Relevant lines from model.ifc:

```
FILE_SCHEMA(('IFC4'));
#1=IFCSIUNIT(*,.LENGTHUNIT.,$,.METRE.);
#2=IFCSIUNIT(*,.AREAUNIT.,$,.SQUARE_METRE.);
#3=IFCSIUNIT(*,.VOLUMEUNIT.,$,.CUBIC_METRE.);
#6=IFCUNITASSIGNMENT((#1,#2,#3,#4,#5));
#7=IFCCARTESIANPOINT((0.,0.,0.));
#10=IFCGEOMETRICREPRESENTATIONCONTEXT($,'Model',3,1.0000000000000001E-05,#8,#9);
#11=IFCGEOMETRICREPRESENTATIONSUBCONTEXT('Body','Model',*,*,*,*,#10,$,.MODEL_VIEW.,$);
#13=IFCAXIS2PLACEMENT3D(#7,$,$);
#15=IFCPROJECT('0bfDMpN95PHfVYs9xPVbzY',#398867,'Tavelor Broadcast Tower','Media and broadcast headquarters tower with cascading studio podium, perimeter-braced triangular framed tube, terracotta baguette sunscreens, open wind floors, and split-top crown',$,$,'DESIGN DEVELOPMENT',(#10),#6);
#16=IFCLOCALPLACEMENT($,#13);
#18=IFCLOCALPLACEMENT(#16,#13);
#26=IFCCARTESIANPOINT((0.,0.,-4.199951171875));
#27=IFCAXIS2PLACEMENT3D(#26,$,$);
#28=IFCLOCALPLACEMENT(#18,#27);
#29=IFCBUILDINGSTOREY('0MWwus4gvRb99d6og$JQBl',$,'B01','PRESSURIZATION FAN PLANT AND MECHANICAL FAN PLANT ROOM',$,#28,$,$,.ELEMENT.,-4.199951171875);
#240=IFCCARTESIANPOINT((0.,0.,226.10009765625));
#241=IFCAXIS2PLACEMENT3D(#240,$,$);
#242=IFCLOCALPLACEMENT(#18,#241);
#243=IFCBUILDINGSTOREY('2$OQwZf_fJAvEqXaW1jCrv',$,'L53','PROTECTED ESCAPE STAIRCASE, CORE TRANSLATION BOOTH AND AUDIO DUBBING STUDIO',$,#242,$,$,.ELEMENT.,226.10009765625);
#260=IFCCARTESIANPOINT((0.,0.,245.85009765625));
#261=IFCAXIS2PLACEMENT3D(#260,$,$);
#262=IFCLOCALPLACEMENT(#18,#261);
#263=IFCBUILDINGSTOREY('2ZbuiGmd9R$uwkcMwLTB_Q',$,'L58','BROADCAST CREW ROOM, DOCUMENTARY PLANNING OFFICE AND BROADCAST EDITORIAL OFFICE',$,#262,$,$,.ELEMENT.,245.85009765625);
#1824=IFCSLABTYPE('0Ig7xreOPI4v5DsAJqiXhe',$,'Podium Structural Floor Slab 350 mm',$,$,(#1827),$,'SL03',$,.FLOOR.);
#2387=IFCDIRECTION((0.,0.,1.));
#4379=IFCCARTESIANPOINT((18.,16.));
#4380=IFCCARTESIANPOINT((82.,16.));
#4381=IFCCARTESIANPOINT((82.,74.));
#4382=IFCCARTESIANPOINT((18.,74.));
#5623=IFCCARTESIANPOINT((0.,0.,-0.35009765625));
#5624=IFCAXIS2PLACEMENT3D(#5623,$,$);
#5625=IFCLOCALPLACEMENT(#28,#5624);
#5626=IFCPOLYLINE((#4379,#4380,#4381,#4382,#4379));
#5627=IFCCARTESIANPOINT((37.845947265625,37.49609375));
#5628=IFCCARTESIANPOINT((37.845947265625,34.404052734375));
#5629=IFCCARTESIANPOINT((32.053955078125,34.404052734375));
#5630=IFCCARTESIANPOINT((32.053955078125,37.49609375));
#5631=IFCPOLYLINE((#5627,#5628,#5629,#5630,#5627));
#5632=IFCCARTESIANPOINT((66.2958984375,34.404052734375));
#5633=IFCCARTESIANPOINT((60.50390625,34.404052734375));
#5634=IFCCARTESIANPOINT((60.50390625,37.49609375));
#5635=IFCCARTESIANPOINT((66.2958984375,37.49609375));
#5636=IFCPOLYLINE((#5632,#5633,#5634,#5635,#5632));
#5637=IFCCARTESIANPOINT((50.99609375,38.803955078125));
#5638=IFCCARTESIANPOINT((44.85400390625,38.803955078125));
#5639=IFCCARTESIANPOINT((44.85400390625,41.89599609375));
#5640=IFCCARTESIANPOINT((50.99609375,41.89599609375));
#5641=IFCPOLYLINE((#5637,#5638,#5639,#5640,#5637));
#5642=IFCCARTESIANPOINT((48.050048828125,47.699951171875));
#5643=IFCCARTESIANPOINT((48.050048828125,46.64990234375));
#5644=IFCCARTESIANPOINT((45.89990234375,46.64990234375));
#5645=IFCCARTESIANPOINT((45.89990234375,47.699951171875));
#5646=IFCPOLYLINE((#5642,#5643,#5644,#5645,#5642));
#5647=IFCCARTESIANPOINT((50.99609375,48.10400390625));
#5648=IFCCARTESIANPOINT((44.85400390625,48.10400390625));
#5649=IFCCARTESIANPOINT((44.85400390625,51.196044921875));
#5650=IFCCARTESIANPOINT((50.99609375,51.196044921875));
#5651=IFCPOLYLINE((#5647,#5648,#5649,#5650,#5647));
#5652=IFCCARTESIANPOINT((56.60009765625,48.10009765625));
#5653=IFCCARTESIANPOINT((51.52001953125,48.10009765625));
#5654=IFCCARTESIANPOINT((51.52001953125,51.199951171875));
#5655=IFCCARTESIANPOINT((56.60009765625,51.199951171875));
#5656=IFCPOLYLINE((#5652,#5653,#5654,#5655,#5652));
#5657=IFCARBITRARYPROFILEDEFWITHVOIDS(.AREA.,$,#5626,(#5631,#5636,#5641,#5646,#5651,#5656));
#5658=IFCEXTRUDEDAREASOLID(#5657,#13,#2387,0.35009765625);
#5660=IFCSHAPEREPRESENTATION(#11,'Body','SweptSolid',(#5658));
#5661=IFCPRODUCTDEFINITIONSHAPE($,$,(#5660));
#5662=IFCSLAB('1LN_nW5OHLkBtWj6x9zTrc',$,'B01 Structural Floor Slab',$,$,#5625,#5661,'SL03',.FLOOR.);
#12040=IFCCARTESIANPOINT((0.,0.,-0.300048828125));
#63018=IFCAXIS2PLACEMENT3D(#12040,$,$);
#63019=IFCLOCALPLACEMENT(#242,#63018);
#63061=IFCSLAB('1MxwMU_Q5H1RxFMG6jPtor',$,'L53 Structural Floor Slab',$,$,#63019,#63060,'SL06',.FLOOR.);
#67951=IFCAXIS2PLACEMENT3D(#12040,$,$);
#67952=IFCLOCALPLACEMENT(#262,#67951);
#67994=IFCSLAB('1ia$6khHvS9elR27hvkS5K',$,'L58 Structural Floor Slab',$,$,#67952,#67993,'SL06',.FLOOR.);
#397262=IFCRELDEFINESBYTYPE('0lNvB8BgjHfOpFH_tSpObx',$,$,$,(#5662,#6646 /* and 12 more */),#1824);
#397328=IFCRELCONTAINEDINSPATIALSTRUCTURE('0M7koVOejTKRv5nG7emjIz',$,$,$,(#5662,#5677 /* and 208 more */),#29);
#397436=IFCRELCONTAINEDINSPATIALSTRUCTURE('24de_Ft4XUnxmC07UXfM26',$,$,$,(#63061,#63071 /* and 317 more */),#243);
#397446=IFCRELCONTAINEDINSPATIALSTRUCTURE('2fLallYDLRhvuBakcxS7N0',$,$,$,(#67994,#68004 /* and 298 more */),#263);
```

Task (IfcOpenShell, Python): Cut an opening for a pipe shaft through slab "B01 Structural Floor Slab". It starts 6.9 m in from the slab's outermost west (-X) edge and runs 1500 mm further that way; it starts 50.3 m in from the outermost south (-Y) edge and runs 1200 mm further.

```python
import numpy as np
import ifcopenshell
import ifcopenshell.api.feature
import ifcopenshell.api.geometry
import ifcopenshell.api.root
import ifcopenshell.geom
import ifcopenshell.util.placement
import ifcopenshell.util.representation
import ifcopenshell.util.shape
import ifcopenshell.util.unit

model = ifcopenshell.open("model.ifc")
unit_scale = ifcopenshell.util.unit.calculate_unit_scale(model)
settings = ifcopenshell.geom.settings()


def volume(element):
    """Net volume in cubic metres, openings subtracted."""
    shape = ifcopenshell.geom.create_shape(settings, element)
    return ifcopenshell.util.shape.get_volume(shape.geometry)


slab = model.by_guid("1LN_nW5OHLkBtWj6x9zTrc")
before = volume(slab)

# Extent in the slab's own axes, in metres. The edges named are its -X and -Y sides.
slab_shape = ifcopenshell.geom.create_shape(settings, slab)
vertices = ifcopenshell.util.shape.get_vertices(slab_shape.geometry)
x_min, y_min, bottom = vertices.min(axis=0)
top = vertices[:, 2].max()

opening = ifcopenshell.api.root.create_entity(model, ifc_class="IfcOpeningElement", name="Pipe shaft opening", predefined_type="OPENING")
context = ifcopenshell.util.representation.get_context(model, "Model", "Body", "MODEL_VIEW")
width, depth = 1.5, 1.2
outline = [(0.0, 0.0), (width, 0.0), (width, depth), (0.0, depth), (0.0, 0.0)]
# Overshoot both faces by 50 mm so the cut is clean.
shape = ifcopenshell.api.geometry.add_slab_representation(
    model, context=context, depth=top - bottom + 0.1, polyline=outline
)
ifcopenshell.api.geometry.assign_representation(model, product=opening, representation=shape)

matrix = ifcopenshell.util.placement.get_local_placement(slab.ObjectPlacement)
matrix[:, 3] = matrix @ np.append(np.array([x_min + 6.9, y_min + 50.3, bottom - 0.05]) / unit_scale, 1.0)
ifcopenshell.api.geometry.edit_object_placement(model, product=opening, matrix=matrix, is_si=False)
ifcopenshell.api.feature.add_feature(model, feature=opening, element=slab)

after = volume(slab)

print(f"slab volume {before:.3f} -> {after:.3f} m3")

model.write("model-out.ifc")
```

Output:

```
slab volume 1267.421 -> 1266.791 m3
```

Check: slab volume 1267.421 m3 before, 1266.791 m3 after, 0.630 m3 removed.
